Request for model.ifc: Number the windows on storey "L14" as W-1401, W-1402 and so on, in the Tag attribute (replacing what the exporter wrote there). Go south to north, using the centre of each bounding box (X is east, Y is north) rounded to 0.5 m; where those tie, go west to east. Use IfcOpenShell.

First a look at what the model holds.

```python
import ifcopenshell
import ifcopenshell.util.element
import ifcopenshell.util.placement

model = ifcopenshell.open("model.ifc")
print(model.schema)
storey = next(s for s in model.by_type("IfcBuildingStorey") if s.Name == "L14")
windows = [e for e in ifcopenshell.util.element.get_decomposition(storey) if e.is_a("IfcWindow")]
for e in sorted(windows, key=lambda e: e.id()):
    origin = ifcopenshell.util.placement.get_local_placement(e.ObjectPlacement)[:3, 3]
    print(e.id(), e.Tag, e.Name, origin.round(2) + 0.0, sep=" | ")
```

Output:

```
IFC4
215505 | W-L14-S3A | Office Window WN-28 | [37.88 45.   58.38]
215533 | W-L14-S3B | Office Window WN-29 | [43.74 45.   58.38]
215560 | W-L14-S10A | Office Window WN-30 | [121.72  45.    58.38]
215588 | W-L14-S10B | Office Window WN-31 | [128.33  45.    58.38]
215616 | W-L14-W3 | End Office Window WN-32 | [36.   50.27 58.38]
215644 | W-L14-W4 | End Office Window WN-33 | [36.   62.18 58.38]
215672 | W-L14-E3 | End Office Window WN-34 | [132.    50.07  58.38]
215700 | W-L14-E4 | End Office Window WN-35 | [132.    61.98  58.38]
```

```python
import ifcopenshell
import ifcopenshell.geom
import ifcopenshell.util.element
import ifcopenshell.util.shape

model = ifcopenshell.open("model.ifc")
settings = ifcopenshell.geom.settings()
settings.set("use-world-coords", True)


def centre(element):
    shape = ifcopenshell.geom.create_shape(settings, element)
    return ifcopenshell.util.shape.get_bbox_centroid(shape.geometry)


storey = next(s for s in model.by_type("IfcBuildingStorey") if s.Name == "L14")
windows = [e for e in ifcopenshell.util.element.get_decomposition(storey) if e.is_a("IfcWindow")]

# Insertion points can sit at a corner or the storey origin, so sort by the geometry (in metres).
centres = {e: centre(e) for e in windows}
windows.sort(key=lambda e: (round(centres[e][1] / 0.5), centres[e][0]))

for i, e in enumerate(windows, start=1):
    number = f"W-14{i:02d}"
    e.Tag = number
    print(e.id(), number)

model.write("model_v2.ifc")
```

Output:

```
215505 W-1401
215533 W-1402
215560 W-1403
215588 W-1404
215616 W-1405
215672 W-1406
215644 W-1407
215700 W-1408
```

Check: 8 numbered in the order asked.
